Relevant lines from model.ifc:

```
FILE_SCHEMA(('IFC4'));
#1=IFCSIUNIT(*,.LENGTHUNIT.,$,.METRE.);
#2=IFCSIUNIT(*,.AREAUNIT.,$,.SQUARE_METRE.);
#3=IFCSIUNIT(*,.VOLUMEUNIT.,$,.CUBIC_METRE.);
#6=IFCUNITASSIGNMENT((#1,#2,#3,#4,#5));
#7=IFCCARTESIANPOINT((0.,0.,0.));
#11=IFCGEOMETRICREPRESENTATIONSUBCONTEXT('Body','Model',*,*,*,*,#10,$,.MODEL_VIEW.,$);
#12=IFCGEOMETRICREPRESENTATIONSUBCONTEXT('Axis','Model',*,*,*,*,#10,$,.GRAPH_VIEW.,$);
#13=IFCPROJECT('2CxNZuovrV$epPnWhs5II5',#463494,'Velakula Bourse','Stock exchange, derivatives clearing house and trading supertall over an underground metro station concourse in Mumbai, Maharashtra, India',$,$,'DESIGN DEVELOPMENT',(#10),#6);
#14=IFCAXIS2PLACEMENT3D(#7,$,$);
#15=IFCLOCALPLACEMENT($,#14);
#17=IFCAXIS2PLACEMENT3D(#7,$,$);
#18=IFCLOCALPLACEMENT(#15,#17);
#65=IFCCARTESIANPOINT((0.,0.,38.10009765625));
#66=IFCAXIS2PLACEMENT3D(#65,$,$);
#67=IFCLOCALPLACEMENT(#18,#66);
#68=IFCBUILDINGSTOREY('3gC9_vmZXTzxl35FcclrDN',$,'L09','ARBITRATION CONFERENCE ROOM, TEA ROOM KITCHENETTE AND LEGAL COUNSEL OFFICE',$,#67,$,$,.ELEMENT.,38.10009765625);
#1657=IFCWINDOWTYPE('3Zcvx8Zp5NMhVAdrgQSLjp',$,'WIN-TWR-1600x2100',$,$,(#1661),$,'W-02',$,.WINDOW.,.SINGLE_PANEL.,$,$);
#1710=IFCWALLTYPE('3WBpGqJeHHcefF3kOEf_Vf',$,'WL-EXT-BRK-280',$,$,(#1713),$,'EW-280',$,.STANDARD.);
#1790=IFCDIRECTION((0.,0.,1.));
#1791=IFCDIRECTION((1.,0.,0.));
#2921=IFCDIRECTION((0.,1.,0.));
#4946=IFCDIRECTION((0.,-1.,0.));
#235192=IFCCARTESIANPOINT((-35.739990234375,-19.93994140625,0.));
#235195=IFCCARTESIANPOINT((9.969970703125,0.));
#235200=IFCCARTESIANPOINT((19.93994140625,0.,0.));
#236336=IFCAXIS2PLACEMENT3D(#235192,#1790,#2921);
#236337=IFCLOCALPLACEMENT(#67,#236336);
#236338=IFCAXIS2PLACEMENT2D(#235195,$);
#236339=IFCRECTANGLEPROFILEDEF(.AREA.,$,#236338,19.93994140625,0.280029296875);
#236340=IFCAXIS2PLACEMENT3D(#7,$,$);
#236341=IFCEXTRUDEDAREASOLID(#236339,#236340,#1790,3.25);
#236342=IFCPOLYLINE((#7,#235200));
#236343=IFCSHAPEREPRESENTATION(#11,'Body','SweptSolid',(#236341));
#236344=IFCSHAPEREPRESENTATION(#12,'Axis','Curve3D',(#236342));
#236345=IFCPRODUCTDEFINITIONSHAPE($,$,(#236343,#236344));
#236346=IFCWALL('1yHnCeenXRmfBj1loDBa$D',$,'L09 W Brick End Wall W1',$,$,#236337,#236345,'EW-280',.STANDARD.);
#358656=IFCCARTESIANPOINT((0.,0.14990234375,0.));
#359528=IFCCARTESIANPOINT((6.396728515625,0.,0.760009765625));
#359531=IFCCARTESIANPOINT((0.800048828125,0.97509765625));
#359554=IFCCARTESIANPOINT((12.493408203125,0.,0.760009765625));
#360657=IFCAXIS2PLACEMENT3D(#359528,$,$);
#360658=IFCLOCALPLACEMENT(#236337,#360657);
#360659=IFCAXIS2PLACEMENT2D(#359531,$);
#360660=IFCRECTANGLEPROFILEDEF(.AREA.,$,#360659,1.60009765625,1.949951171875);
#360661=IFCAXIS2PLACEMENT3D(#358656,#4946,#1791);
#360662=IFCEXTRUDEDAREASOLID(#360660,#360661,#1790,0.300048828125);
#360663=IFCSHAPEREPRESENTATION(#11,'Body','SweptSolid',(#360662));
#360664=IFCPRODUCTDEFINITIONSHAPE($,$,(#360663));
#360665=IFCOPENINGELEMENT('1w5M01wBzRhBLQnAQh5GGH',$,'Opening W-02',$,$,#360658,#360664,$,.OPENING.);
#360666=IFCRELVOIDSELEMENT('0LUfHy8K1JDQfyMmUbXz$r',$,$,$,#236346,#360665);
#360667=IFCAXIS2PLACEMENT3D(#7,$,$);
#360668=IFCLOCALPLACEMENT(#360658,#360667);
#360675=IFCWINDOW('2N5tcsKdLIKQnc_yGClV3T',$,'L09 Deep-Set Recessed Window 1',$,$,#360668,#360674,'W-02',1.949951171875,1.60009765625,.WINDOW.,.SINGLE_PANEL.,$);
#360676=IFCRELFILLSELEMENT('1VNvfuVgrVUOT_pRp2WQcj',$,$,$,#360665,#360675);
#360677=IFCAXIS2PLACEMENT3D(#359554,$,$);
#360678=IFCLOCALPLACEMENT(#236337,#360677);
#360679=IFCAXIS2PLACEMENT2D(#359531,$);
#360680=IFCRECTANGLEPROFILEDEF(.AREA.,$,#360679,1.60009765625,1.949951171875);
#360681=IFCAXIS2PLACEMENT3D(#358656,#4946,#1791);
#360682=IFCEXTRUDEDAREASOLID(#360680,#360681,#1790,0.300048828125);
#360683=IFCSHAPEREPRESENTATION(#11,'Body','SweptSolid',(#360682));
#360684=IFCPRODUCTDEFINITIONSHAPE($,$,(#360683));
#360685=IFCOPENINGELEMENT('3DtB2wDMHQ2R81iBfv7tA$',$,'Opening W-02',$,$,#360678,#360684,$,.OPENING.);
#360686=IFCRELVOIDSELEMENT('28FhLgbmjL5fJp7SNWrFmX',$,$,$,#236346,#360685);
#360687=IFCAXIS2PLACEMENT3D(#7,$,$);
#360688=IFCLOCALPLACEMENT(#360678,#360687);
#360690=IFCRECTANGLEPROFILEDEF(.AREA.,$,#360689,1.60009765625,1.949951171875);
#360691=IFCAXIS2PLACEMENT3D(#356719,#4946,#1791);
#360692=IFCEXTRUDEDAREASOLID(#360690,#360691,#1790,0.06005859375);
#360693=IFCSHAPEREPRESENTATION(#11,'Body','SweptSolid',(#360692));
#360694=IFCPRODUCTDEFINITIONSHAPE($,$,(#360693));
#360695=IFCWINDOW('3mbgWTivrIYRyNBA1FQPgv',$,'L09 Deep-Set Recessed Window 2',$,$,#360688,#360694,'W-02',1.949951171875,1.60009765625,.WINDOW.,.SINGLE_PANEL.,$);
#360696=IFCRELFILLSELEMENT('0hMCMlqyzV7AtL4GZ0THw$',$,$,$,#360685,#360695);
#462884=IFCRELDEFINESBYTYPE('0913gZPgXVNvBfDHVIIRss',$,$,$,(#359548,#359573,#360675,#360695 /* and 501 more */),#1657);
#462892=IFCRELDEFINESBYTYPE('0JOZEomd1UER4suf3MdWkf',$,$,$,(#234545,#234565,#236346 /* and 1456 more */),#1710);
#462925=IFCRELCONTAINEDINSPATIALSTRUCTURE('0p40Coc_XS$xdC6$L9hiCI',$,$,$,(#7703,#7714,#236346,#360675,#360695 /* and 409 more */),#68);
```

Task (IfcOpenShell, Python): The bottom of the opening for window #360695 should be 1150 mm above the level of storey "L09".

```python
import numpy as np
import ifcopenshell
import ifcopenshell.api.geometry
import ifcopenshell.geom
import ifcopenshell.util.element
import ifcopenshell.util.placement
import ifcopenshell.util.shape
import ifcopenshell.util.unit

model = ifcopenshell.open("model.ifc")
unit_scale = ifcopenshell.util.unit.calculate_unit_scale(model)

window = model.by_guid("3mbgWTivrIYRyNBA1FQPgv")
opening = window.FillsVoids[0].RelatingOpeningElement
storey = ifcopenshell.util.element.get_container(window, ifc_class="IfcBuildingStorey")
level = ifcopenshell.util.placement.get_local_placement(storey.ObjectPlacement)[2, 3]

# The opening's origin need not be at the sill, so measure its lowest point.
shape = ifcopenshell.geom.create_shape(ifcopenshell.geom.settings(), opening)
bottom = ifcopenshell.util.shape.get_shape_bottom_elevation(shape, shape.geometry) / unit_scale
dz = level + 1.15 / unit_scale - bottom

shift = np.array([0.0, 0.0, dz])
# The window is placed relative to its opening, so it follows when the opening moves.
matrix = ifcopenshell.util.placement.get_local_placement(opening.ObjectPlacement)
matrix[:3, 3] += shift
ifcopenshell.api.geometry.edit_object_placement(
    model, product=opening, matrix=matrix, is_si=False, should_transform_children=True
)

print(f"moved by {dz * unit_scale:+.3f} m")

model.write("model_v2.ifc")
```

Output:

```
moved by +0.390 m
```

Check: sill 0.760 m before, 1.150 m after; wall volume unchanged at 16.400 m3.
